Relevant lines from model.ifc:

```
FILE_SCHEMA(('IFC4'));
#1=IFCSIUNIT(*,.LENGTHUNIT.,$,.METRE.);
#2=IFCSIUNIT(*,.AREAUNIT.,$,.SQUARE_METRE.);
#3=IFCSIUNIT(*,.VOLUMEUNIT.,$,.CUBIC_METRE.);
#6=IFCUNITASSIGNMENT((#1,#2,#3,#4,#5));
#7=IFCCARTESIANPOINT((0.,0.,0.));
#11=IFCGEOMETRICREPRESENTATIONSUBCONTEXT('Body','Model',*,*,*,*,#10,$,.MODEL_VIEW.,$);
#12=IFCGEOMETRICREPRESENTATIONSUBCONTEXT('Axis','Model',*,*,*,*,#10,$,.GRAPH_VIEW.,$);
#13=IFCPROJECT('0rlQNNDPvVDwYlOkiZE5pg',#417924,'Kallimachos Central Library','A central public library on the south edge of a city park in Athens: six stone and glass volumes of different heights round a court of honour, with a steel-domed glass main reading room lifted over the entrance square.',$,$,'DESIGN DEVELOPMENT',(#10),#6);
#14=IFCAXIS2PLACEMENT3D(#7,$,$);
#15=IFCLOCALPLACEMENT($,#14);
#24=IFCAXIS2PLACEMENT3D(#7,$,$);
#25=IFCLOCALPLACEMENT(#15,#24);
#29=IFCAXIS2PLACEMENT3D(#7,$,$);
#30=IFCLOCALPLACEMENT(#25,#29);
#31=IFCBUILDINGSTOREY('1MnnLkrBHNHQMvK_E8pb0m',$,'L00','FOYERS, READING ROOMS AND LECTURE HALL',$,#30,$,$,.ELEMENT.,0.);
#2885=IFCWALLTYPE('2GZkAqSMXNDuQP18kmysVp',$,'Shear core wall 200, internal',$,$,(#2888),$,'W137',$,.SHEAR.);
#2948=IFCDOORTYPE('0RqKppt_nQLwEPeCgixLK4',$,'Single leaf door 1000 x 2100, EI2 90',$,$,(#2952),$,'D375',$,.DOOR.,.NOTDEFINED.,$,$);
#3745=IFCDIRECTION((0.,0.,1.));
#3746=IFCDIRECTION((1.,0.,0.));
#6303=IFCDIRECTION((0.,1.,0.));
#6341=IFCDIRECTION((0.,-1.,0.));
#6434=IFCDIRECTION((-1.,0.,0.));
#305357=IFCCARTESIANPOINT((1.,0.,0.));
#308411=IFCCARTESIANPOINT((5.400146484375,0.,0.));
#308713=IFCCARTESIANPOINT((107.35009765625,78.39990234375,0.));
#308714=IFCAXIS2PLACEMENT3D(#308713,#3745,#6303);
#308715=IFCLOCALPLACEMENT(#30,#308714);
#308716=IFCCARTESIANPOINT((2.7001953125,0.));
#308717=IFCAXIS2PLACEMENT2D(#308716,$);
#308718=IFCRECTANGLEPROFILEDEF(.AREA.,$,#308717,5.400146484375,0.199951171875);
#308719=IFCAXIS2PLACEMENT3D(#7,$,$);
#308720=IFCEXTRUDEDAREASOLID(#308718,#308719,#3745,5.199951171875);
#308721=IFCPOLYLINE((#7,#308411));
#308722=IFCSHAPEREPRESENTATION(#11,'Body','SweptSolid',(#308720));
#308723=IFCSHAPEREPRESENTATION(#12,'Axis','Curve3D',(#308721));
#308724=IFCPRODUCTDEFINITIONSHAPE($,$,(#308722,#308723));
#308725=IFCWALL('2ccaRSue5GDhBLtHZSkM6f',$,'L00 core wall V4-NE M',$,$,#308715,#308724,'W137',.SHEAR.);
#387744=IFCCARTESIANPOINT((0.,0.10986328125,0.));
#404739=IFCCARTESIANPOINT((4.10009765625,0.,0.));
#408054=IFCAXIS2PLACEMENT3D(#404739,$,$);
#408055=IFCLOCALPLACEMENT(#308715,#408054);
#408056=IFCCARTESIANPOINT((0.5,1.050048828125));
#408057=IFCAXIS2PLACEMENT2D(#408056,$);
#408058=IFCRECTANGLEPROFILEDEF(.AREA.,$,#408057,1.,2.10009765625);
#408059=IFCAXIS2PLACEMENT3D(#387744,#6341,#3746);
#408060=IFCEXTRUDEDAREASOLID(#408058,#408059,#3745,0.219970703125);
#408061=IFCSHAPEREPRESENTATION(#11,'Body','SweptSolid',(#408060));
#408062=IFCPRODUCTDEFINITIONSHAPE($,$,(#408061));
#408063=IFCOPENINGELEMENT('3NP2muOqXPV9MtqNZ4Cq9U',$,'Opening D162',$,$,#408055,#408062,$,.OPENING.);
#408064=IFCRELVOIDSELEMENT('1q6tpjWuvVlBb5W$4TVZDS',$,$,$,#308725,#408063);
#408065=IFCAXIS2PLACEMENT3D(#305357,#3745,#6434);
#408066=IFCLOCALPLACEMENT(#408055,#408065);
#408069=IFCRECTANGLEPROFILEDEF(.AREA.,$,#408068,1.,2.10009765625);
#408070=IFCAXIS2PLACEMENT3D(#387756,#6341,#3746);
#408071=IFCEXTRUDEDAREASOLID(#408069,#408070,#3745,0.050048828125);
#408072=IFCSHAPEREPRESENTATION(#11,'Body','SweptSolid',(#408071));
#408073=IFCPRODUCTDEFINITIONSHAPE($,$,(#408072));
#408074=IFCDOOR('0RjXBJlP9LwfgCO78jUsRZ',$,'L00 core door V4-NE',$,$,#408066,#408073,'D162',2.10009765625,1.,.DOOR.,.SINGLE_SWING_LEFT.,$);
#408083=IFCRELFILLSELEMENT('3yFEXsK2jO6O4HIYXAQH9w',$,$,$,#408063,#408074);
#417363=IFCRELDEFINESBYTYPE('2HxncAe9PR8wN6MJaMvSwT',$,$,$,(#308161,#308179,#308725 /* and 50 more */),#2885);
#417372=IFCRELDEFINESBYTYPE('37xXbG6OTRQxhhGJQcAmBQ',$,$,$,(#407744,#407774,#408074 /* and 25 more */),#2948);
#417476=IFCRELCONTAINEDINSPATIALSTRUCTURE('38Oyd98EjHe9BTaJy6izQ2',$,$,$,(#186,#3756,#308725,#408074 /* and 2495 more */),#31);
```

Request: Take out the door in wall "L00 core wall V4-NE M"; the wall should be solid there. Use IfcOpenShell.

```python
import ifcopenshell
import ifcopenshell.api.feature
import ifcopenshell.api.root
import ifcopenshell.geom
import ifcopenshell.util.shape

model = ifcopenshell.open("model.ifc")
settings = ifcopenshell.geom.settings()


def volume(element):
    """Net volume in cubic metres, openings subtracted."""
    shape = ifcopenshell.geom.create_shape(settings, element)
    return ifcopenshell.util.shape.get_volume(shape.geometry)


door = model.by_id(408074)
opening = door.FillsVoids[0].RelatingOpeningElement
wall = opening.VoidsElements[0].RelatingBuildingElement
before = volume(wall)

ifcopenshell.api.root.remove_product(model, product=door)
ifcopenshell.api.feature.remove_feature(model, feature=opening)

after = volume(wall)

print(f"wall volume {before:.3f} -> {after:.3f} m3")

model.write("model-out.ifc")
```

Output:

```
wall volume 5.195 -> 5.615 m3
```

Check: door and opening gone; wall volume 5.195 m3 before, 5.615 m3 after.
